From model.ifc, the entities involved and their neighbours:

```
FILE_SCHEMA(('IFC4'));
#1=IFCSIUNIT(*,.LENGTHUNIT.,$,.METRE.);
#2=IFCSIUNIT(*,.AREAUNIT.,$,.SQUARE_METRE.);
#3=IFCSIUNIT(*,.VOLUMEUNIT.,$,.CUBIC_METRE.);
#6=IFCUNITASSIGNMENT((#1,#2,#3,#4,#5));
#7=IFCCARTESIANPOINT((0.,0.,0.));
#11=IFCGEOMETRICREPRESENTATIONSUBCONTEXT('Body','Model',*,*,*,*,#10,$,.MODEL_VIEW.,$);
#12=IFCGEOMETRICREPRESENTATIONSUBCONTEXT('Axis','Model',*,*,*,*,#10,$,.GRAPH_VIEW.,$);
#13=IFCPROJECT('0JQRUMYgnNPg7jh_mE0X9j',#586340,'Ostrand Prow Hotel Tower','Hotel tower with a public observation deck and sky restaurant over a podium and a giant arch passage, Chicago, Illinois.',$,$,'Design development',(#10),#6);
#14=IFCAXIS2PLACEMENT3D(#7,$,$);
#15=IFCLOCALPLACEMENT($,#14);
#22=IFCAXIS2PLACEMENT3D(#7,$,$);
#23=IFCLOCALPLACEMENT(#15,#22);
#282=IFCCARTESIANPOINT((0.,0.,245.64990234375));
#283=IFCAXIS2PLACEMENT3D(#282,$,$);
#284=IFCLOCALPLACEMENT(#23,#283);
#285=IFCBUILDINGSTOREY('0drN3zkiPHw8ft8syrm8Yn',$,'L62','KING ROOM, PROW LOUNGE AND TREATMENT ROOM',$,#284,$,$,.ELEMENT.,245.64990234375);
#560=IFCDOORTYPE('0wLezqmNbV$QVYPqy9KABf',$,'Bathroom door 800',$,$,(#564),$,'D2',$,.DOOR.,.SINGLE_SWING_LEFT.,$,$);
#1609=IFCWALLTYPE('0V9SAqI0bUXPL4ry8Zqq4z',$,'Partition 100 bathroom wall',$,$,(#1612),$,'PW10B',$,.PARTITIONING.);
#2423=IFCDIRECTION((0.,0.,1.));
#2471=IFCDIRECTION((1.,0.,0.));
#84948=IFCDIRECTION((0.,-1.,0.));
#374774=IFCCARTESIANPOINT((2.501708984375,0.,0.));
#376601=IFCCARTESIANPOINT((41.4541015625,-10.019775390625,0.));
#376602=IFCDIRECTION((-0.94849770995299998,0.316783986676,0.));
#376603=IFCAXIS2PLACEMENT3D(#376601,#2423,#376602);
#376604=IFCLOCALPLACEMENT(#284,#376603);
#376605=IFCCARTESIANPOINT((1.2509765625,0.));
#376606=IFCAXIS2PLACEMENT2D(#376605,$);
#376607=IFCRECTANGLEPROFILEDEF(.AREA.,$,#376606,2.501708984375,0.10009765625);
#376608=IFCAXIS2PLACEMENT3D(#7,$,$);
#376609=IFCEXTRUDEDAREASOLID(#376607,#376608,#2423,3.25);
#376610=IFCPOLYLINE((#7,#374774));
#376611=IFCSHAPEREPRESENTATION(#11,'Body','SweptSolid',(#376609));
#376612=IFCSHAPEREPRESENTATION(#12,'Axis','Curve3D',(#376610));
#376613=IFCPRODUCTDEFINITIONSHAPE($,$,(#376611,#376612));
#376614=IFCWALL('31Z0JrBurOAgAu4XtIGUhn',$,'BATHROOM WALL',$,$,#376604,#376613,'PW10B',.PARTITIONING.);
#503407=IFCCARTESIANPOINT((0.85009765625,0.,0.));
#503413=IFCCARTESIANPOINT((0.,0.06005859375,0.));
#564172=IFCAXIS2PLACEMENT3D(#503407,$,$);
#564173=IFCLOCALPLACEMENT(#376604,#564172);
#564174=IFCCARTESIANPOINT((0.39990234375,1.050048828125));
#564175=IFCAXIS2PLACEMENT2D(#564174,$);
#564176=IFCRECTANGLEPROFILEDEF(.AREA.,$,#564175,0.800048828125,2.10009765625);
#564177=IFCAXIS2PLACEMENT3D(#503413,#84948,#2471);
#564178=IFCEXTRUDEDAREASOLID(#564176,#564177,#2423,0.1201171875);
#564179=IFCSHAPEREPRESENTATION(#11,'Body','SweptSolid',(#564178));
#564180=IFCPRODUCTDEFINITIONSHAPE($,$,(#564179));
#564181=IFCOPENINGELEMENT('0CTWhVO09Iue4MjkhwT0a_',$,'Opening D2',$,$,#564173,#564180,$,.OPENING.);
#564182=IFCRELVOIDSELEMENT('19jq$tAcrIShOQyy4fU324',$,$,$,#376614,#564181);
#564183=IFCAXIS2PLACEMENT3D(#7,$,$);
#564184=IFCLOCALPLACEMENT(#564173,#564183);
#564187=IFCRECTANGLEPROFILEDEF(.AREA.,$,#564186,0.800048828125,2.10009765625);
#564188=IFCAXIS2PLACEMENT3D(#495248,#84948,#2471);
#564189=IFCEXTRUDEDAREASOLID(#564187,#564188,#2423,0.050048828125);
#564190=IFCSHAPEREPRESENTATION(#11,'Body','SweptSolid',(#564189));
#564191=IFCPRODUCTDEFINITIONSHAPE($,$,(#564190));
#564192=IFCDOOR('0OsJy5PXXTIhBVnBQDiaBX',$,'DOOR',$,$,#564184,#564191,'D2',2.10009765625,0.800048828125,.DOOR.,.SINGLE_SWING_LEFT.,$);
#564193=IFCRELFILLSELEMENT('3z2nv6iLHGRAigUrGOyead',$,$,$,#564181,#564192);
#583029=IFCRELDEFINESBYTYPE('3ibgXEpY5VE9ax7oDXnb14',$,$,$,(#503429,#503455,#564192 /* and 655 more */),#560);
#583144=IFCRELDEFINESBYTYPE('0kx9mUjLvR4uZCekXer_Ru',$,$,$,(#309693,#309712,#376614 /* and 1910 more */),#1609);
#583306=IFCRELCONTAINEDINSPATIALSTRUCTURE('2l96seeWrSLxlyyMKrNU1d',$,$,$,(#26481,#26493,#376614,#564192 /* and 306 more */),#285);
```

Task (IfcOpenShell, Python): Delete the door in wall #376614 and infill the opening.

```python
import ifcopenshell
import ifcopenshell.api.feature
import ifcopenshell.api.root
import ifcopenshell.geom
import ifcopenshell.util.shape

model = ifcopenshell.open("model.ifc")
settings = ifcopenshell.geom.settings()


def volume(element):
    """Net volume in cubic metres, openings subtracted."""
    shape = ifcopenshell.geom.create_shape(settings, element)
    return ifcopenshell.util.shape.get_volume(shape.geometry)


door = model.by_guid("0OsJy5PXXTIhBVnBQDiaBX")
opening = door.FillsVoids[0].RelatingOpeningElement
wall = opening.VoidsElements[0].RelatingBuildingElement
before = volume(wall)

ifcopenshell.api.root.remove_product(model, product=door)
ifcopenshell.api.feature.remove_feature(model, feature=opening)

after = volume(wall)

print(f"wall volume {before:.3f} -> {after:.3f} m3")

model.write("model_updated.ifc")
```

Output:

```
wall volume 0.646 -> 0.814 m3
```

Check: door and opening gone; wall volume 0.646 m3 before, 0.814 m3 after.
